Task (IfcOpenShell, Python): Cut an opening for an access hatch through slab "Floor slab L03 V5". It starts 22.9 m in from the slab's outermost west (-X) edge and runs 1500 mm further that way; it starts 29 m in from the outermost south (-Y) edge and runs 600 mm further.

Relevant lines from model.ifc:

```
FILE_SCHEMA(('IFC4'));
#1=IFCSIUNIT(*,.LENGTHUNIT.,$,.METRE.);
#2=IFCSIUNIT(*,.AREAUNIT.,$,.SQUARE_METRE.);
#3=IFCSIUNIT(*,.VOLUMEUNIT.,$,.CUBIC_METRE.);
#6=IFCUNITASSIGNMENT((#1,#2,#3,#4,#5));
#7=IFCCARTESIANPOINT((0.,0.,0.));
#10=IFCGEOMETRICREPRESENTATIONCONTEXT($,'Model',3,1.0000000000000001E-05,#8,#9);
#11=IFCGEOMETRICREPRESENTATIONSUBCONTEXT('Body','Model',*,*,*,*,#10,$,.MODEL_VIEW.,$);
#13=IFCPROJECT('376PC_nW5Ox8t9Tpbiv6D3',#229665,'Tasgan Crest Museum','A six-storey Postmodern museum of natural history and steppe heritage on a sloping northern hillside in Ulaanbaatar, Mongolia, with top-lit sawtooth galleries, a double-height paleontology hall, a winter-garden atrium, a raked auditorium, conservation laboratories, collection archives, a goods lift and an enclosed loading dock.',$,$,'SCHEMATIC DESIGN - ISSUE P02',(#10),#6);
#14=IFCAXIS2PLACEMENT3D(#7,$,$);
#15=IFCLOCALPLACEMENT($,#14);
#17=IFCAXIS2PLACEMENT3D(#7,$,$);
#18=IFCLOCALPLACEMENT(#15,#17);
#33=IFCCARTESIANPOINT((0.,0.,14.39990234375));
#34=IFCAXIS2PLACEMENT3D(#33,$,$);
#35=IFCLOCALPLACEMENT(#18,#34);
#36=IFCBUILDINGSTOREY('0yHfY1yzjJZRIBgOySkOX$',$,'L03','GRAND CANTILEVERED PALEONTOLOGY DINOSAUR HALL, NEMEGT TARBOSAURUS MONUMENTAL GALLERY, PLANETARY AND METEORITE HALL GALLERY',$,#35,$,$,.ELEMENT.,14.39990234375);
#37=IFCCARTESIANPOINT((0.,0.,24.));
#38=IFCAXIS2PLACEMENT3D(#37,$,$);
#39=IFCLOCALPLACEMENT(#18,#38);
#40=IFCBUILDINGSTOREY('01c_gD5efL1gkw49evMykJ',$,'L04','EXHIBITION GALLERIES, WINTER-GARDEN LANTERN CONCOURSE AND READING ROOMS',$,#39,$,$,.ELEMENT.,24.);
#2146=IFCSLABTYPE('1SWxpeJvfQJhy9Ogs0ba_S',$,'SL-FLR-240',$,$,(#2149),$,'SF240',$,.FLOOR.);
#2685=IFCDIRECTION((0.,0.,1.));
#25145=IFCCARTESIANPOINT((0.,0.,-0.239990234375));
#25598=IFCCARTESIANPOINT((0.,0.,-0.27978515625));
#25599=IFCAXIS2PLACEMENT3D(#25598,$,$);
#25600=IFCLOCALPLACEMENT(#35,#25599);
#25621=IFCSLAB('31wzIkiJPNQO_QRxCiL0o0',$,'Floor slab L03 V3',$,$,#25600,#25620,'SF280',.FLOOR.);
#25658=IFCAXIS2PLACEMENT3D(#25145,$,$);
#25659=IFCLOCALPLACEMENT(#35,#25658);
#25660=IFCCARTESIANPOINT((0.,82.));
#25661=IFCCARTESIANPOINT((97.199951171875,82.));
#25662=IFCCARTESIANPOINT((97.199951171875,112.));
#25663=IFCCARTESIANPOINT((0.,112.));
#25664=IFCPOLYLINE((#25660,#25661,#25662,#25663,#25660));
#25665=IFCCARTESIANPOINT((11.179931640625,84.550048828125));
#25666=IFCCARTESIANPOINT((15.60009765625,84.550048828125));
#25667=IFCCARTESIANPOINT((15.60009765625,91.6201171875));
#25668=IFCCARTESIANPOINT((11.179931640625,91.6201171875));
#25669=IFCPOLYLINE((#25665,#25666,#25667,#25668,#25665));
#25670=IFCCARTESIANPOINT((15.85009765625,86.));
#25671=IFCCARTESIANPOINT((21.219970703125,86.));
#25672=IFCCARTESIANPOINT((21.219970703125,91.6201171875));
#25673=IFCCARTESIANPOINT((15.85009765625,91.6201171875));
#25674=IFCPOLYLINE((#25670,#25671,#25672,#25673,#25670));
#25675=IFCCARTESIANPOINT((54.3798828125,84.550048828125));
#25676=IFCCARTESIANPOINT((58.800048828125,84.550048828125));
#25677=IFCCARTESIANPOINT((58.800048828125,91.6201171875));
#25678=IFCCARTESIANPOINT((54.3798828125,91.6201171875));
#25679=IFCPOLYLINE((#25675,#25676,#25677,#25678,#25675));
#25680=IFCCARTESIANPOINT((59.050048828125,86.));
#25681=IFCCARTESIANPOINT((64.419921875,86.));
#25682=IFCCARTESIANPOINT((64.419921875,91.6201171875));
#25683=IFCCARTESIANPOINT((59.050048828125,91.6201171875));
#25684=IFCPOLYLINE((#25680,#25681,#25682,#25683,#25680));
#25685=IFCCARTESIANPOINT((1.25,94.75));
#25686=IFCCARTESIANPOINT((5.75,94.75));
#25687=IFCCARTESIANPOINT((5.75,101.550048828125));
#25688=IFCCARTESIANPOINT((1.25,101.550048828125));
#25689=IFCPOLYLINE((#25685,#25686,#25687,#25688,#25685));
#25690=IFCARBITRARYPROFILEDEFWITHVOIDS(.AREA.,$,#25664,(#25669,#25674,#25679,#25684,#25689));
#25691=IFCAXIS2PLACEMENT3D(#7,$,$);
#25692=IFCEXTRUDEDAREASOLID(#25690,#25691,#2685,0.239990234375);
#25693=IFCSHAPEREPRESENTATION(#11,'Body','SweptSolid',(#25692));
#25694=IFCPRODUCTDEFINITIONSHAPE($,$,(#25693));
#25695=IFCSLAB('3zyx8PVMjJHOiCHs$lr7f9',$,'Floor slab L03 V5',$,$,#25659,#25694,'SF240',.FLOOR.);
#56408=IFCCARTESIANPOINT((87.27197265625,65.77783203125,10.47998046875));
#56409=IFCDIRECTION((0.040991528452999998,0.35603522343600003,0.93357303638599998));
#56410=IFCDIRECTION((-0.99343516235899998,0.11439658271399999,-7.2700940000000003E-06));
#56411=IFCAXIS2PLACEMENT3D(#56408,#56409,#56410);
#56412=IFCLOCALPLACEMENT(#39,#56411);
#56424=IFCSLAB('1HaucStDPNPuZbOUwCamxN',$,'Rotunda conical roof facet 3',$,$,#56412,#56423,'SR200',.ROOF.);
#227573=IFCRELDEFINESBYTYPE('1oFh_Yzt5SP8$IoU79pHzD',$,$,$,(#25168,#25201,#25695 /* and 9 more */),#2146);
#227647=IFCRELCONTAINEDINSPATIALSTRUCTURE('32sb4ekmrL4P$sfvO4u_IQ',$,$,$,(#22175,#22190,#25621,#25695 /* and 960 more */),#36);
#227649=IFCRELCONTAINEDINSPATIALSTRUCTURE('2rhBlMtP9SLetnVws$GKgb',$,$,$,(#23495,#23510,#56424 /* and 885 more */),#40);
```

```python
import numpy as np
import ifcopenshell
import ifcopenshell.api.feature
import ifcopenshell.api.geometry
import ifcopenshell.api.root
import ifcopenshell.geom
import ifcopenshell.util.placement
import ifcopenshell.util.representation
import ifcopenshell.util.shape
import ifcopenshell.util.unit

model = ifcopenshell.open("model.ifc")
unit_scale = ifcopenshell.util.unit.calculate_unit_scale(model)
settings = ifcopenshell.geom.settings()


def volume(element):
    """Net volume in cubic metres, openings subtracted."""
    shape = ifcopenshell.geom.create_shape(settings, element)
    return ifcopenshell.util.shape.get_volume(shape.geometry)


slab = model.by_guid("3zyx8PVMjJHOiCHs$lr7f9")
before = volume(slab)

# Extent in the slab's own axes, in metres. The edges named are its -X and -Y sides.
slab_shape = ifcopenshell.geom.create_shape(settings, slab)
vertices = ifcopenshell.util.shape.get_vertices(slab_shape.geometry)
x_min, y_min, bottom = vertices.min(axis=0)
top = vertices[:, 2].max()

opening = ifcopenshell.api.root.create_entity(model, ifc_class="IfcOpeningElement", name="Access hatch opening", predefined_type="OPENING")
context = ifcopenshell.util.representation.get_context(model, "Model", "Body", "MODEL_VIEW")
width, depth = 1.5, 0.6
outline = [(0.0, 0.0), (width, 0.0), (width, depth), (0.0, depth), (0.0, 0.0)]
# Overshoot both faces by 50 mm so the cut is clean.
shape = ifcopenshell.api.geometry.add_slab_representation(
    model, context=context, depth=top - bottom + 0.1, polyline=outline
)
ifcopenshell.api.geometry.assign_representation(model, product=opening, representation=shape)

matrix = ifcopenshell.util.placement.get_local_placement(slab.ObjectPlacement)
matrix[:, 3] = matrix @ np.append(np.array([x_min + 22.9, y_min + 29, bottom - 0.05]) / unit_scale, 1.0)
ifcopenshell.api.geometry.edit_object_placement(model, product=opening, matrix=matrix, is_si=False)
ifcopenshell.api.feature.add_feature(model, feature=opening, element=slab)

after = volume(slab)

print(f"slab volume {before:.3f} -> {after:.3f} m3")

model.write("model_v2.ifc")
```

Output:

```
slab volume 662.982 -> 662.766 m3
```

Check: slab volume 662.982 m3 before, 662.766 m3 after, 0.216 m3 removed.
